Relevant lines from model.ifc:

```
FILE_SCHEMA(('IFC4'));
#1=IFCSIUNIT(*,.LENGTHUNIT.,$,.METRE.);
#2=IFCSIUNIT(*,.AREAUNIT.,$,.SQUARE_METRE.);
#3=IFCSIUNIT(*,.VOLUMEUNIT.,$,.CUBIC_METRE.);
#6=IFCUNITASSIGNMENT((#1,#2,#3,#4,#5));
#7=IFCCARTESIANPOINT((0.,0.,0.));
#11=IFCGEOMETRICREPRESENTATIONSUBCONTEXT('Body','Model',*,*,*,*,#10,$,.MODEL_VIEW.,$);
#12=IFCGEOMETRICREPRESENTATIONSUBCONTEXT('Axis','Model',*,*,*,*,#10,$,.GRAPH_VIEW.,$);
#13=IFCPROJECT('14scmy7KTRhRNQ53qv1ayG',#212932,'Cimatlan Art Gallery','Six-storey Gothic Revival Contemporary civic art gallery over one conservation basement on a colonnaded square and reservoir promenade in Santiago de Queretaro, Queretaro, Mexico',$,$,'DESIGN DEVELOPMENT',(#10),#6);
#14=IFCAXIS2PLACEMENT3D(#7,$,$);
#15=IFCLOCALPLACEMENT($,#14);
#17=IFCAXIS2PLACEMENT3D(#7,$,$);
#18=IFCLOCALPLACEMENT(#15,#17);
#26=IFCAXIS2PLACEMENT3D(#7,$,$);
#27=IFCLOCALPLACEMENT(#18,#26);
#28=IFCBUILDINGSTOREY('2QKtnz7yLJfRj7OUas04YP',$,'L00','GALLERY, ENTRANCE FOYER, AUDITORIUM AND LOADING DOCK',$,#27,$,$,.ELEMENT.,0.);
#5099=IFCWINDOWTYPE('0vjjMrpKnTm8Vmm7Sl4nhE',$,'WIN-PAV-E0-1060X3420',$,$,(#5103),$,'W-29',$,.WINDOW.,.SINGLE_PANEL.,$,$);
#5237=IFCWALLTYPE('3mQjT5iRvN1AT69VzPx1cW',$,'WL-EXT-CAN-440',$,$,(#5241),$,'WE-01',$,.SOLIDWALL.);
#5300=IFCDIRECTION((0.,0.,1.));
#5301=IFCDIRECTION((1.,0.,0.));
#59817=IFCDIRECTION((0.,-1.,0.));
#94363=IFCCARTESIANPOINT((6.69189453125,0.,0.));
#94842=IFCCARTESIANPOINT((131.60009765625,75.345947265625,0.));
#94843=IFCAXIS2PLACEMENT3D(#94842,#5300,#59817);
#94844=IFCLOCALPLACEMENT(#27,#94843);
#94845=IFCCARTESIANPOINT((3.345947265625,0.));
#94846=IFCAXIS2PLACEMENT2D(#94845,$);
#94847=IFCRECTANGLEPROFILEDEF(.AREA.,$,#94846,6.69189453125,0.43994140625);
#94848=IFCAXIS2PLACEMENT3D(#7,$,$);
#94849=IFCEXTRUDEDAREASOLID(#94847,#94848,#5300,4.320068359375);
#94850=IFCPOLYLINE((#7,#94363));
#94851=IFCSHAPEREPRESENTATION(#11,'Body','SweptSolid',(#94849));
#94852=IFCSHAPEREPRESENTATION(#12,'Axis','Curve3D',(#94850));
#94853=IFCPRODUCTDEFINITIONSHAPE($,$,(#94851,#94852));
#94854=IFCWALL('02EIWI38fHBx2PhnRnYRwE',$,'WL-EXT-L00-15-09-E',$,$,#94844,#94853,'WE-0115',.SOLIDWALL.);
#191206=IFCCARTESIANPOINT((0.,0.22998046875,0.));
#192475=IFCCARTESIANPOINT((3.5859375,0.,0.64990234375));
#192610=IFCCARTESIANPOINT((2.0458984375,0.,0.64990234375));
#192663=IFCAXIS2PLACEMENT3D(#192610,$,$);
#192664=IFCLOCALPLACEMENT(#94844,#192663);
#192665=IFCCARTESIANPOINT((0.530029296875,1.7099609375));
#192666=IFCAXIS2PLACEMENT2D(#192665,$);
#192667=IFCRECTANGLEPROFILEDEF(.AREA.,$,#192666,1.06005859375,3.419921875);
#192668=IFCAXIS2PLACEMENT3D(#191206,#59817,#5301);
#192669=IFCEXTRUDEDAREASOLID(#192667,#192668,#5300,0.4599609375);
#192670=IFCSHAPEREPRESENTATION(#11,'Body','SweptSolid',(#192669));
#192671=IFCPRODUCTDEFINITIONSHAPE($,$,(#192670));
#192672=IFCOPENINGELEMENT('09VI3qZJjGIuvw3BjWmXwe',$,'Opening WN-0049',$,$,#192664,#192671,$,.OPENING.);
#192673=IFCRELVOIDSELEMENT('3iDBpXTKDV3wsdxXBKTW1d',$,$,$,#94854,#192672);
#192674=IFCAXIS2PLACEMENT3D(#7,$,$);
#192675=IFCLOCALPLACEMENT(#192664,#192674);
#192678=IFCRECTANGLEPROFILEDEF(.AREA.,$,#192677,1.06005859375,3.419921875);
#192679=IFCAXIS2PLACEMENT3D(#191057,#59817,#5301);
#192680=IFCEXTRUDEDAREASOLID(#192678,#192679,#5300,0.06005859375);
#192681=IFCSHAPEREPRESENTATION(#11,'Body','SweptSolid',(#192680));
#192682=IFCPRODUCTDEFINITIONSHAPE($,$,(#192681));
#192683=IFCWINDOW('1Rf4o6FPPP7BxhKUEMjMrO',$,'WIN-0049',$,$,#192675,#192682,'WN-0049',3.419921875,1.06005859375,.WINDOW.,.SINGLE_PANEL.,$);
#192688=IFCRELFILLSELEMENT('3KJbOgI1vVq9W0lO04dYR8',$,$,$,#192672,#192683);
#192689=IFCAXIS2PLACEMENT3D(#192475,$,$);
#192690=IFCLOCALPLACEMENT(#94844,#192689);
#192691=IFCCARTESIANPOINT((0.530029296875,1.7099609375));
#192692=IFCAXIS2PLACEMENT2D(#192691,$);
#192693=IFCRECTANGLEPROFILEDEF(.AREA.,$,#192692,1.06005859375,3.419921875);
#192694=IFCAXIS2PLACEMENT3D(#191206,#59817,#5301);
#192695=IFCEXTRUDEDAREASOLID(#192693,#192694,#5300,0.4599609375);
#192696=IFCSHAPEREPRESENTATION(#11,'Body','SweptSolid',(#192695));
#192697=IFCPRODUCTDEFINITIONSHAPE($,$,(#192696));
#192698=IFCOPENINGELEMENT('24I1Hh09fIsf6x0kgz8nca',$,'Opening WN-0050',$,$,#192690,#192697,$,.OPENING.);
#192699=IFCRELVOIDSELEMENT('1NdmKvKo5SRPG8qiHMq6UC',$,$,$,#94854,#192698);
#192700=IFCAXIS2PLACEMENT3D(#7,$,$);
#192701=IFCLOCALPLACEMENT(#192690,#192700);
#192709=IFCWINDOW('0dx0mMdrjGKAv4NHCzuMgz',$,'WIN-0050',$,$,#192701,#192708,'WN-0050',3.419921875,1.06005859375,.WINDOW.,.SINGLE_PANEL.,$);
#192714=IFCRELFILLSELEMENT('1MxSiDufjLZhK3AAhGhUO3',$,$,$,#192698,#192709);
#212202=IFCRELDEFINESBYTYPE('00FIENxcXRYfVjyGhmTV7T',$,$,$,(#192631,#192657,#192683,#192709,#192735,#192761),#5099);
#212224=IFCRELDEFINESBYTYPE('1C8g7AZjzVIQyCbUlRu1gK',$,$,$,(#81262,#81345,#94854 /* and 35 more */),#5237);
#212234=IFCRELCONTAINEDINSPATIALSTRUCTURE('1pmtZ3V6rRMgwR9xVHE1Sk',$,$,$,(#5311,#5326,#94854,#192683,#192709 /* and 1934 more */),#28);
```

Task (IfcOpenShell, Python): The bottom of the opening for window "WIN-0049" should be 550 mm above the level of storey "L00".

```python
import numpy as np
import ifcopenshell
import ifcopenshell.api.geometry
import ifcopenshell.geom
import ifcopenshell.util.element
import ifcopenshell.util.placement
import ifcopenshell.util.shape
import ifcopenshell.util.unit

model = ifcopenshell.open("model.ifc")
unit_scale = ifcopenshell.util.unit.calculate_unit_scale(model)

window = model.by_id(192683)
opening = window.FillsVoids[0].RelatingOpeningElement
storey = ifcopenshell.util.element.get_container(window, ifc_class="IfcBuildingStorey")
level = ifcopenshell.util.placement.get_local_placement(storey.ObjectPlacement)[2, 3]

# The opening's origin need not be at the sill, so measure its lowest point.
shape = ifcopenshell.geom.create_shape(ifcopenshell.geom.settings(), opening)
bottom = ifcopenshell.util.shape.get_shape_bottom_elevation(shape, shape.geometry) / unit_scale
dz = level + 0.55 / unit_scale - bottom

shift = np.array([0.0, 0.0, dz])
# The window is placed relative to its opening, so it follows when the opening moves.
matrix = ifcopenshell.util.placement.get_local_placement(opening.ObjectPlacement)
matrix[:3, 3] += shift
ifcopenshell.api.geometry.edit_object_placement(
    model, product=opening, matrix=matrix, is_si=False, should_transform_children=True
)

print(f"moved by {dz * unit_scale:+.3f} m")

model.write("model_updated.ifc")
```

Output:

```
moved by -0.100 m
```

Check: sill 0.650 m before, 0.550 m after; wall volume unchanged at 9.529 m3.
